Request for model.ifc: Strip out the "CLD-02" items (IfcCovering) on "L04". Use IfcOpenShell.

First a look at what the model holds.

```python
import ifcopenshell
import ifcopenshell.util.element

model = ifcopenshell.open("model.ifc")
print(model.schema)
storey = next(s for s in model.by_type("IfcBuildingStorey") if s.Name == "L04")
coverings = [e for e in ifcopenshell.util.element.get_decomposition(storey) if e.is_a("IfcCovering")]
seen = {}
for e in coverings:
    element_type = ifcopenshell.util.element.get_type(e)
    name = element_type.Name if element_type not in (None, e) else None
    seen[name] = seen.get(name, 0) + 1
for name, count in sorted(seen.items(), key=str):
    print(count, "x", name)
```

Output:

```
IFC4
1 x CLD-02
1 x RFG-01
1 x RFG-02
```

```python
import ifcopenshell
import ifcopenshell.api.root
import ifcopenshell.util.element

model = ifcopenshell.open("model.ifc")

storey = next(s for s in model.by_type("IfcBuildingStorey") if s.Name == "L04")
coverings = [e for e in ifcopenshell.util.element.get_decomposition(storey) if e.is_a("IfcCovering")]
targets = [e for e in coverings if (t := ifcopenshell.util.element.get_type(e)) not in (None, e) and t.Name == "CLD-02"]

for e in targets:
    ifcopenshell.api.root.remove_product(model, product=e)
print(len(targets), "removed")

model.write("model_updated.ifc")
```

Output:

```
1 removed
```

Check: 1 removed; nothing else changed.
